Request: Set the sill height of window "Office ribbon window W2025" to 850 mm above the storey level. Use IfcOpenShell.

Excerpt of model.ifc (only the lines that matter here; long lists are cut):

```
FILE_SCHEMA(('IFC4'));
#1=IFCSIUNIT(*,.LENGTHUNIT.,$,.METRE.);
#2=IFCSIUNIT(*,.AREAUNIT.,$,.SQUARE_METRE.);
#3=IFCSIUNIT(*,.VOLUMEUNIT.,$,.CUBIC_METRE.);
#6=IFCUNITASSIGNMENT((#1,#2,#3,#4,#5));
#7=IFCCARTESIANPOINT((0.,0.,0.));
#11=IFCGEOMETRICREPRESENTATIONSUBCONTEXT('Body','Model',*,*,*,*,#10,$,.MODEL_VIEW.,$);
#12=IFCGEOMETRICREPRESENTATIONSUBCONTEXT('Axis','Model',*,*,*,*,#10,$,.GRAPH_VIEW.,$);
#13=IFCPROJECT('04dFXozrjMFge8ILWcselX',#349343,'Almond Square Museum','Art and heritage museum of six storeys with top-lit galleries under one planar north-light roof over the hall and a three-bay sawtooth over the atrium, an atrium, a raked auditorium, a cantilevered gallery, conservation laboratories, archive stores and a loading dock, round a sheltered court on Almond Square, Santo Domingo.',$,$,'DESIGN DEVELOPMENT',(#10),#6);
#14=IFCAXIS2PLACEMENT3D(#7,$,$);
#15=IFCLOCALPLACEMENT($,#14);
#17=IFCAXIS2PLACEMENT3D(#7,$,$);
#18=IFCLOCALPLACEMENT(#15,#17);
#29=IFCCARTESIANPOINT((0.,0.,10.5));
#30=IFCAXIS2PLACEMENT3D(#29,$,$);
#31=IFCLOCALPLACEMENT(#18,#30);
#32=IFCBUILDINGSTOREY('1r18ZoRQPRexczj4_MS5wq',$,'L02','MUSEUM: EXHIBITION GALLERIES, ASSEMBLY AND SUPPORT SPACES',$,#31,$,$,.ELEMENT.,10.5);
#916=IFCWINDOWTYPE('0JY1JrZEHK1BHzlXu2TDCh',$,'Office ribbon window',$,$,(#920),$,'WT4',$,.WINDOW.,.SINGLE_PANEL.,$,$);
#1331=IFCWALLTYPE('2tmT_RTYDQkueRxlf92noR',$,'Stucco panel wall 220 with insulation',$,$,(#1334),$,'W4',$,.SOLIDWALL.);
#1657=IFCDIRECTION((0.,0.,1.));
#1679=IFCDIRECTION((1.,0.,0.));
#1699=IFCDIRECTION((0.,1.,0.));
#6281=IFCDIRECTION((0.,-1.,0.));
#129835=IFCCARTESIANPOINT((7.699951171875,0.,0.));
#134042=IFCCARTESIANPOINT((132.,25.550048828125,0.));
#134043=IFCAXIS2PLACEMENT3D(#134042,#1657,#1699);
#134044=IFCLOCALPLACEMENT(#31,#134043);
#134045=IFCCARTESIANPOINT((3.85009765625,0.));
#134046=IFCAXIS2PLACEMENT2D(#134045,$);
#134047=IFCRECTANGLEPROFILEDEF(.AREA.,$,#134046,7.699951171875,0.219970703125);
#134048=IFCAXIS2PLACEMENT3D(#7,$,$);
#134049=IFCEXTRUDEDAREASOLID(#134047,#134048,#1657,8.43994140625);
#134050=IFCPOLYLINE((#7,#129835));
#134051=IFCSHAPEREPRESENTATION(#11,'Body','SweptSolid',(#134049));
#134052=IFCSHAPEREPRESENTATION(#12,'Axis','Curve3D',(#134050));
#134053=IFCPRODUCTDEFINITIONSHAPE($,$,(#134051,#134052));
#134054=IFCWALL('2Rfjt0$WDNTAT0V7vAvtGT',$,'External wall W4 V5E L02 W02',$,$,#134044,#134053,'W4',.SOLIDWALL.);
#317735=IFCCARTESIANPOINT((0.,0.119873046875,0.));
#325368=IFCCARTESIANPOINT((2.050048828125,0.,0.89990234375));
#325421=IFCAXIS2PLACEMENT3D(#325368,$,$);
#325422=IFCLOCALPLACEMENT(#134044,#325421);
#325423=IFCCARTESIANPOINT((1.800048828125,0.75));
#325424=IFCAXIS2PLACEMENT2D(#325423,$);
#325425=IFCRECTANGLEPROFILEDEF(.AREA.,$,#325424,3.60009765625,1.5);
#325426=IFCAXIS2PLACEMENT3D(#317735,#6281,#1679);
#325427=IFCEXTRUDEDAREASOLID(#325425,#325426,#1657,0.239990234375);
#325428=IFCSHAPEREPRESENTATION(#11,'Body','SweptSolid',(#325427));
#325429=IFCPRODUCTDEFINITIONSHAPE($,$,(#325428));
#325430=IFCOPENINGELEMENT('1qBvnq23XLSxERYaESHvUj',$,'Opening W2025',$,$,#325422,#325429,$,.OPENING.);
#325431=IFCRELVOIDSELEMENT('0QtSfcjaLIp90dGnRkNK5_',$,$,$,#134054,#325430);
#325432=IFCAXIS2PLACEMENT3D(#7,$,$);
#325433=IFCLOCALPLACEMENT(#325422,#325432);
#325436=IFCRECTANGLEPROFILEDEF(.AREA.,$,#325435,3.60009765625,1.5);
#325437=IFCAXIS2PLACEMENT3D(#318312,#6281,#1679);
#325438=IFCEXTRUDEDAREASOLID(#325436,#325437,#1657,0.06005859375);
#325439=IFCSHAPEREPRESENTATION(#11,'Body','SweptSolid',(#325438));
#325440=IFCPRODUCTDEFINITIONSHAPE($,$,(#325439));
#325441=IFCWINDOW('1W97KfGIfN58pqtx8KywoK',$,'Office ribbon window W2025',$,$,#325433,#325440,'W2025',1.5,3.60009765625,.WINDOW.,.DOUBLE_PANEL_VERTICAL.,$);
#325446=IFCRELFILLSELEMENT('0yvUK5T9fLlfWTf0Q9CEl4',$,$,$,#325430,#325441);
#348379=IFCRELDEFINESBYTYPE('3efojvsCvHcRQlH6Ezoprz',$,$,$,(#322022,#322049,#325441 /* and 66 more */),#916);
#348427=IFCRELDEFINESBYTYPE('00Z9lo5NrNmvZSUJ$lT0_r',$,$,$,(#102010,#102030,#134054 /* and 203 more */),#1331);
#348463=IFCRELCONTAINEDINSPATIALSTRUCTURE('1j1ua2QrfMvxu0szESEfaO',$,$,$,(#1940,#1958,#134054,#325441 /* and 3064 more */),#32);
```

```python
import numpy as np
import ifcopenshell
import ifcopenshell.api.geometry
import ifcopenshell.geom
import ifcopenshell.util.element
import ifcopenshell.util.placement
import ifcopenshell.util.shape
import ifcopenshell.util.unit

model = ifcopenshell.open("model.ifc")
unit_scale = ifcopenshell.util.unit.calculate_unit_scale(model)

window = model.by_id(325441)
opening = window.FillsVoids[0].RelatingOpeningElement
storey = ifcopenshell.util.element.get_container(window, ifc_class="IfcBuildingStorey")
level = ifcopenshell.util.placement.get_local_placement(storey.ObjectPlacement)[2, 3]

# The opening's origin need not be at the sill, so measure its lowest point.
shape = ifcopenshell.geom.create_shape(ifcopenshell.geom.settings(), opening)
bottom = ifcopenshell.util.shape.get_shape_bottom_elevation(shape, shape.geometry) / unit_scale
dz = level + 0.85 - bottom

shift = np.array([0.0, 0.0, dz])
# The window is placed relative to its opening, so it follows when the opening moves.
matrix = ifcopenshell.util.placement.get_local_placement(opening.ObjectPlacement)
matrix[:3, 3] += shift
ifcopenshell.api.geometry.edit_object_placement(
    model, product=opening, matrix=matrix, is_si=False, should_transform_children=True
)

print(f"moved by {dz * unit_scale:+.3f} m")

model.write("model_edited.ifc")
```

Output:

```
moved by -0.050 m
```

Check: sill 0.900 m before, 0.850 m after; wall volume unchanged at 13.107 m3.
